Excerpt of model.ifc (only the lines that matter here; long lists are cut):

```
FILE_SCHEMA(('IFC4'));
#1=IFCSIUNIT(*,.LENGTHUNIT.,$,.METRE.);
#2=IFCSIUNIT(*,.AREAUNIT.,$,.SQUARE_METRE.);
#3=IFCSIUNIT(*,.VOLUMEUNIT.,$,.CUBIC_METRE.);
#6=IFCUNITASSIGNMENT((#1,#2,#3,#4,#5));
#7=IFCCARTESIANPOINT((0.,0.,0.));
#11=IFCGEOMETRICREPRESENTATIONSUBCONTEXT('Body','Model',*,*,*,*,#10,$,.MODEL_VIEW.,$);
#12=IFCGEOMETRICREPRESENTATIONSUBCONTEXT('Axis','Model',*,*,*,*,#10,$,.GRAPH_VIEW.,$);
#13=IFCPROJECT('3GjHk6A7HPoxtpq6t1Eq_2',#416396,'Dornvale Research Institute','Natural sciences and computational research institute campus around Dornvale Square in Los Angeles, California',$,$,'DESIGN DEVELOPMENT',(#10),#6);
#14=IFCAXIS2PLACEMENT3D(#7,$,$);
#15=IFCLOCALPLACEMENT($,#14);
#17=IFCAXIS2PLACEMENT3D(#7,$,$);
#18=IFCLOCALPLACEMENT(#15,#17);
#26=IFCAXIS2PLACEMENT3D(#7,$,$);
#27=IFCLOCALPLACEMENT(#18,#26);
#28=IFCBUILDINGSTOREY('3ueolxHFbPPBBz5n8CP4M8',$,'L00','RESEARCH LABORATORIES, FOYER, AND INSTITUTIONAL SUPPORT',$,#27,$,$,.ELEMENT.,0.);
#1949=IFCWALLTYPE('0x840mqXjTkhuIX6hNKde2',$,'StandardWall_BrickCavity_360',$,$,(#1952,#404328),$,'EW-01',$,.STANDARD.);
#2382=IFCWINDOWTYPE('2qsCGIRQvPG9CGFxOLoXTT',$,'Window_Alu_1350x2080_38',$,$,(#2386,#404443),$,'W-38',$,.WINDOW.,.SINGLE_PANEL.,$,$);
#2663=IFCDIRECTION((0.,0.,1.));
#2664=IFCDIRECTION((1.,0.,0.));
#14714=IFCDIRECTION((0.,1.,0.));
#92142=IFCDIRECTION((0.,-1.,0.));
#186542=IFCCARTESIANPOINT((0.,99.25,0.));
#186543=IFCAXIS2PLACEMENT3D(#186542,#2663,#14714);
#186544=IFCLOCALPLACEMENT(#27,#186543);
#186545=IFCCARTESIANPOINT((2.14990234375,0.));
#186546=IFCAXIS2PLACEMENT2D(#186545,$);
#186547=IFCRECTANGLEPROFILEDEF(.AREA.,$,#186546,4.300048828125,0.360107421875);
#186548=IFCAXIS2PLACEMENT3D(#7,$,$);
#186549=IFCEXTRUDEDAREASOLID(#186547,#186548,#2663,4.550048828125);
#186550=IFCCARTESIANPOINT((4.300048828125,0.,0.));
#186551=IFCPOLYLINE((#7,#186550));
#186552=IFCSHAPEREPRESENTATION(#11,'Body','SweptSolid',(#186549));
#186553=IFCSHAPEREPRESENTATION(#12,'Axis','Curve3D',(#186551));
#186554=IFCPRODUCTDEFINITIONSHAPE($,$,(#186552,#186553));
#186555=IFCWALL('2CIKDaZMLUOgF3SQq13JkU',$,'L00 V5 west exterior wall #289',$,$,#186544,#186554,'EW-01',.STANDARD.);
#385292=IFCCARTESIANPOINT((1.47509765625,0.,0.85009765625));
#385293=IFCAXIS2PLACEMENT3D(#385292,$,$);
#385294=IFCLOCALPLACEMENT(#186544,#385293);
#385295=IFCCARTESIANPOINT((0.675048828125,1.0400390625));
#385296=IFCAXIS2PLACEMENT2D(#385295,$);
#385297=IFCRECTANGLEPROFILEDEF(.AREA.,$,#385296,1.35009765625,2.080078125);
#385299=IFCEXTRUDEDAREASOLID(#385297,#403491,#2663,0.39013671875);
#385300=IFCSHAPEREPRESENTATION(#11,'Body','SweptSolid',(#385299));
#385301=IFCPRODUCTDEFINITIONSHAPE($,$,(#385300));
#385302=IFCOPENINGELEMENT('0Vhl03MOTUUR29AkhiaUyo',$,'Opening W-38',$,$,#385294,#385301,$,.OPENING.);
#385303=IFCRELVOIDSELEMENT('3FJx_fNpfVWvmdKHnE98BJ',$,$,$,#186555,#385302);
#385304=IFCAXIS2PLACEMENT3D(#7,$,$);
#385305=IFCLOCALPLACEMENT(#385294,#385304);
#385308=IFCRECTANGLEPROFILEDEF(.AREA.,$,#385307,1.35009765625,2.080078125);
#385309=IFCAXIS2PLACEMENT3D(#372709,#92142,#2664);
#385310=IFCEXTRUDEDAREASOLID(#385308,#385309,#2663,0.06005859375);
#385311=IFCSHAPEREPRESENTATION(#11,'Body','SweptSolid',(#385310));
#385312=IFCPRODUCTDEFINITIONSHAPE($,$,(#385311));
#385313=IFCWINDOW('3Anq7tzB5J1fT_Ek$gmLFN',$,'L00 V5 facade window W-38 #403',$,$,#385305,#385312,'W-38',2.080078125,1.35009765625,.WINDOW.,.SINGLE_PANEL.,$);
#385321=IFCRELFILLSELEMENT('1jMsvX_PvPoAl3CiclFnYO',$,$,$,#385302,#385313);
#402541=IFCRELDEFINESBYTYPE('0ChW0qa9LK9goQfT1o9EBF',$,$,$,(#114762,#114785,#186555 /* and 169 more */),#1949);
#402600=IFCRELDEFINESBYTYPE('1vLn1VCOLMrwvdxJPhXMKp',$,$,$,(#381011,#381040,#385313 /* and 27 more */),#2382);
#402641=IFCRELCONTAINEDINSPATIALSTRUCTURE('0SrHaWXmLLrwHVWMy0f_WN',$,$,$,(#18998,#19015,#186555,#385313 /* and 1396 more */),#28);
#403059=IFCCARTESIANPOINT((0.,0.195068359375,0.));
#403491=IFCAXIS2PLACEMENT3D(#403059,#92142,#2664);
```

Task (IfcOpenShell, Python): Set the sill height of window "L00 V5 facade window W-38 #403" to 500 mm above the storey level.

```python
import numpy as np
import ifcopenshell
import ifcopenshell.api.geometry
import ifcopenshell.geom
import ifcopenshell.util.element
import ifcopenshell.util.placement
import ifcopenshell.util.shape
import ifcopenshell.util.unit

model = ifcopenshell.open("model.ifc")
unit_scale = ifcopenshell.util.unit.calculate_unit_scale(model)

window = model.by_id(385313)
opening = window.FillsVoids[0].RelatingOpeningElement
storey = ifcopenshell.util.element.get_container(window, ifc_class="IfcBuildingStorey")
level = ifcopenshell.util.placement.get_local_placement(storey.ObjectPlacement)[2, 3]

# The opening's origin need not be at the sill, so measure its lowest point.
shape = ifcopenshell.geom.create_shape(ifcopenshell.geom.settings(), opening)
bottom = ifcopenshell.util.shape.get_shape_bottom_elevation(shape, shape.geometry) / unit_scale
dz = level + 0.5 - bottom

shift = np.array([0.0, 0.0, dz])
# The window is placed relative to its opening, so it follows when the opening moves.
matrix = ifcopenshell.util.placement.get_local_placement(opening.ObjectPlacement)
matrix[:3, 3] += shift
ifcopenshell.api.geometry.edit_object_placement(
    model, product=opening, matrix=matrix, is_si=False, should_transform_children=True
)

print(f"moved by {dz * unit_scale:+.3f} m")

model.write("model_rev.ifc")
```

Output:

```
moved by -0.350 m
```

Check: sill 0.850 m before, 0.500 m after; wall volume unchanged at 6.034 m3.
